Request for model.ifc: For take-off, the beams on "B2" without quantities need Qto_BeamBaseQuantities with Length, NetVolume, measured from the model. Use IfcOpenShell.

First a look at what the model holds.

```python
import ifcopenshell
import ifcopenshell.util.element
import ifcopenshell.util.unit

model = ifcopenshell.open("model.ifc")
print(model.schema)
for unit_type in ("LENGTHUNIT", "AREAUNIT", "VOLUMEUNIT"):
    print(unit_type, ifcopenshell.util.unit.calculate_unit_scale(model, unit_type))
storey = next(s for s in model.by_type("IfcBuildingStorey") if s.Name == "B2")
beams = [e for e in ifcopenshell.util.element.get_decomposition(storey) if e.is_a("IfcBeam")]
for e in sorted(beams, key=lambda e: e.id()):
    print(e.id(), e.is_a(), e.Name, list(ifcopenshell.util.element.get_psets(e, qtos_only=True)), sep=" | ")
```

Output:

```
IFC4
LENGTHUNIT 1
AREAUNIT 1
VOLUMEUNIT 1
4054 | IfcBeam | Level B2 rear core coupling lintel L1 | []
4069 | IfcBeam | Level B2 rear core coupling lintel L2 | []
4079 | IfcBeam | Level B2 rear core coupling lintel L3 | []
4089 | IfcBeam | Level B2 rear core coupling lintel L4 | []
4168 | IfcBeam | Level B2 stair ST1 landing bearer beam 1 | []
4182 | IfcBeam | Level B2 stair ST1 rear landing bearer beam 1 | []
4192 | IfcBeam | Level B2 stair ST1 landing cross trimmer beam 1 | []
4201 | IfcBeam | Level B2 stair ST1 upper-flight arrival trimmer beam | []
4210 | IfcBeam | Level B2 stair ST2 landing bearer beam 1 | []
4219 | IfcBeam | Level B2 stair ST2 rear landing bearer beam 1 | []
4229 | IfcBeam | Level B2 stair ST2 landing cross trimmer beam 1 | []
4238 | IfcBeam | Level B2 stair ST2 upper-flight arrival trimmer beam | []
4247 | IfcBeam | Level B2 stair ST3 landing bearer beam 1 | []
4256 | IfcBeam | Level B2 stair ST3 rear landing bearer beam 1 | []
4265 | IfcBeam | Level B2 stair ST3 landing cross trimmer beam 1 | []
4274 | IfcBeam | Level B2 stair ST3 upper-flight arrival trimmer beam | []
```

```python
import ifcopenshell
import ifcopenshell.api.pset
import ifcopenshell.geom
import ifcopenshell.util.element
import ifcopenshell.util.shape
import ifcopenshell.util.unit

model = ifcopenshell.open("model.ifc")
unit_scale = ifcopenshell.util.unit.calculate_unit_scale(model)
volume_scale = ifcopenshell.util.unit.calculate_unit_scale(model, "VOLUMEUNIT")
settings = ifcopenshell.geom.settings()

storey = next(s for s in model.by_type("IfcBuildingStorey") if s.Name == "B2")
beams = [e for e in ifcopenshell.util.element.get_decomposition(storey) if e.is_a("IfcBeam")]

for e in sorted(beams, key=lambda e: e.id()):
    if ifcopenshell.util.element.get_psets(e, qtos_only=True, should_inherit=False):
        continue
    # Geometry comes back in metres, in the element's own axes.
    shape = ifcopenshell.geom.create_shape(settings, e)
    values = {
        "Length": ifcopenshell.util.shape.get_max_xyz(shape.geometry) / unit_scale,
        "NetVolume": ifcopenshell.util.shape.get_volume(shape.geometry) / volume_scale,
    }
    qto = ifcopenshell.api.pset.add_qto(model, product=e, name="Qto_BeamBaseQuantities")
    ifcopenshell.api.pset.edit_qto(model, qto=qto, properties=values)
    print(e.id(), {k: round(v, 3) for k, v in values.items()})

model.write("model_rev.ifc")
```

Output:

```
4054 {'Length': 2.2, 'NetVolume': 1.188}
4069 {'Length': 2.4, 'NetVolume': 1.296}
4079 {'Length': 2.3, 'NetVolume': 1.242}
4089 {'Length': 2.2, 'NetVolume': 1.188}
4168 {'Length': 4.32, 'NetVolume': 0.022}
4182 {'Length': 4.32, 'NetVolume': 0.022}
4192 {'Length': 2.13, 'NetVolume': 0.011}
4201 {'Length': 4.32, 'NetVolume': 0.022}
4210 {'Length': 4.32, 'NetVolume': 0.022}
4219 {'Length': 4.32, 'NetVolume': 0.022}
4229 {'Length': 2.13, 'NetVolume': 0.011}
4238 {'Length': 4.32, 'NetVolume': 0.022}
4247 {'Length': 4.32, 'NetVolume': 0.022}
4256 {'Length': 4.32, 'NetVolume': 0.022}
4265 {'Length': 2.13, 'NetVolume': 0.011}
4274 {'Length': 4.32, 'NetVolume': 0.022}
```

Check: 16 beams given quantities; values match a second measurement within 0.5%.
